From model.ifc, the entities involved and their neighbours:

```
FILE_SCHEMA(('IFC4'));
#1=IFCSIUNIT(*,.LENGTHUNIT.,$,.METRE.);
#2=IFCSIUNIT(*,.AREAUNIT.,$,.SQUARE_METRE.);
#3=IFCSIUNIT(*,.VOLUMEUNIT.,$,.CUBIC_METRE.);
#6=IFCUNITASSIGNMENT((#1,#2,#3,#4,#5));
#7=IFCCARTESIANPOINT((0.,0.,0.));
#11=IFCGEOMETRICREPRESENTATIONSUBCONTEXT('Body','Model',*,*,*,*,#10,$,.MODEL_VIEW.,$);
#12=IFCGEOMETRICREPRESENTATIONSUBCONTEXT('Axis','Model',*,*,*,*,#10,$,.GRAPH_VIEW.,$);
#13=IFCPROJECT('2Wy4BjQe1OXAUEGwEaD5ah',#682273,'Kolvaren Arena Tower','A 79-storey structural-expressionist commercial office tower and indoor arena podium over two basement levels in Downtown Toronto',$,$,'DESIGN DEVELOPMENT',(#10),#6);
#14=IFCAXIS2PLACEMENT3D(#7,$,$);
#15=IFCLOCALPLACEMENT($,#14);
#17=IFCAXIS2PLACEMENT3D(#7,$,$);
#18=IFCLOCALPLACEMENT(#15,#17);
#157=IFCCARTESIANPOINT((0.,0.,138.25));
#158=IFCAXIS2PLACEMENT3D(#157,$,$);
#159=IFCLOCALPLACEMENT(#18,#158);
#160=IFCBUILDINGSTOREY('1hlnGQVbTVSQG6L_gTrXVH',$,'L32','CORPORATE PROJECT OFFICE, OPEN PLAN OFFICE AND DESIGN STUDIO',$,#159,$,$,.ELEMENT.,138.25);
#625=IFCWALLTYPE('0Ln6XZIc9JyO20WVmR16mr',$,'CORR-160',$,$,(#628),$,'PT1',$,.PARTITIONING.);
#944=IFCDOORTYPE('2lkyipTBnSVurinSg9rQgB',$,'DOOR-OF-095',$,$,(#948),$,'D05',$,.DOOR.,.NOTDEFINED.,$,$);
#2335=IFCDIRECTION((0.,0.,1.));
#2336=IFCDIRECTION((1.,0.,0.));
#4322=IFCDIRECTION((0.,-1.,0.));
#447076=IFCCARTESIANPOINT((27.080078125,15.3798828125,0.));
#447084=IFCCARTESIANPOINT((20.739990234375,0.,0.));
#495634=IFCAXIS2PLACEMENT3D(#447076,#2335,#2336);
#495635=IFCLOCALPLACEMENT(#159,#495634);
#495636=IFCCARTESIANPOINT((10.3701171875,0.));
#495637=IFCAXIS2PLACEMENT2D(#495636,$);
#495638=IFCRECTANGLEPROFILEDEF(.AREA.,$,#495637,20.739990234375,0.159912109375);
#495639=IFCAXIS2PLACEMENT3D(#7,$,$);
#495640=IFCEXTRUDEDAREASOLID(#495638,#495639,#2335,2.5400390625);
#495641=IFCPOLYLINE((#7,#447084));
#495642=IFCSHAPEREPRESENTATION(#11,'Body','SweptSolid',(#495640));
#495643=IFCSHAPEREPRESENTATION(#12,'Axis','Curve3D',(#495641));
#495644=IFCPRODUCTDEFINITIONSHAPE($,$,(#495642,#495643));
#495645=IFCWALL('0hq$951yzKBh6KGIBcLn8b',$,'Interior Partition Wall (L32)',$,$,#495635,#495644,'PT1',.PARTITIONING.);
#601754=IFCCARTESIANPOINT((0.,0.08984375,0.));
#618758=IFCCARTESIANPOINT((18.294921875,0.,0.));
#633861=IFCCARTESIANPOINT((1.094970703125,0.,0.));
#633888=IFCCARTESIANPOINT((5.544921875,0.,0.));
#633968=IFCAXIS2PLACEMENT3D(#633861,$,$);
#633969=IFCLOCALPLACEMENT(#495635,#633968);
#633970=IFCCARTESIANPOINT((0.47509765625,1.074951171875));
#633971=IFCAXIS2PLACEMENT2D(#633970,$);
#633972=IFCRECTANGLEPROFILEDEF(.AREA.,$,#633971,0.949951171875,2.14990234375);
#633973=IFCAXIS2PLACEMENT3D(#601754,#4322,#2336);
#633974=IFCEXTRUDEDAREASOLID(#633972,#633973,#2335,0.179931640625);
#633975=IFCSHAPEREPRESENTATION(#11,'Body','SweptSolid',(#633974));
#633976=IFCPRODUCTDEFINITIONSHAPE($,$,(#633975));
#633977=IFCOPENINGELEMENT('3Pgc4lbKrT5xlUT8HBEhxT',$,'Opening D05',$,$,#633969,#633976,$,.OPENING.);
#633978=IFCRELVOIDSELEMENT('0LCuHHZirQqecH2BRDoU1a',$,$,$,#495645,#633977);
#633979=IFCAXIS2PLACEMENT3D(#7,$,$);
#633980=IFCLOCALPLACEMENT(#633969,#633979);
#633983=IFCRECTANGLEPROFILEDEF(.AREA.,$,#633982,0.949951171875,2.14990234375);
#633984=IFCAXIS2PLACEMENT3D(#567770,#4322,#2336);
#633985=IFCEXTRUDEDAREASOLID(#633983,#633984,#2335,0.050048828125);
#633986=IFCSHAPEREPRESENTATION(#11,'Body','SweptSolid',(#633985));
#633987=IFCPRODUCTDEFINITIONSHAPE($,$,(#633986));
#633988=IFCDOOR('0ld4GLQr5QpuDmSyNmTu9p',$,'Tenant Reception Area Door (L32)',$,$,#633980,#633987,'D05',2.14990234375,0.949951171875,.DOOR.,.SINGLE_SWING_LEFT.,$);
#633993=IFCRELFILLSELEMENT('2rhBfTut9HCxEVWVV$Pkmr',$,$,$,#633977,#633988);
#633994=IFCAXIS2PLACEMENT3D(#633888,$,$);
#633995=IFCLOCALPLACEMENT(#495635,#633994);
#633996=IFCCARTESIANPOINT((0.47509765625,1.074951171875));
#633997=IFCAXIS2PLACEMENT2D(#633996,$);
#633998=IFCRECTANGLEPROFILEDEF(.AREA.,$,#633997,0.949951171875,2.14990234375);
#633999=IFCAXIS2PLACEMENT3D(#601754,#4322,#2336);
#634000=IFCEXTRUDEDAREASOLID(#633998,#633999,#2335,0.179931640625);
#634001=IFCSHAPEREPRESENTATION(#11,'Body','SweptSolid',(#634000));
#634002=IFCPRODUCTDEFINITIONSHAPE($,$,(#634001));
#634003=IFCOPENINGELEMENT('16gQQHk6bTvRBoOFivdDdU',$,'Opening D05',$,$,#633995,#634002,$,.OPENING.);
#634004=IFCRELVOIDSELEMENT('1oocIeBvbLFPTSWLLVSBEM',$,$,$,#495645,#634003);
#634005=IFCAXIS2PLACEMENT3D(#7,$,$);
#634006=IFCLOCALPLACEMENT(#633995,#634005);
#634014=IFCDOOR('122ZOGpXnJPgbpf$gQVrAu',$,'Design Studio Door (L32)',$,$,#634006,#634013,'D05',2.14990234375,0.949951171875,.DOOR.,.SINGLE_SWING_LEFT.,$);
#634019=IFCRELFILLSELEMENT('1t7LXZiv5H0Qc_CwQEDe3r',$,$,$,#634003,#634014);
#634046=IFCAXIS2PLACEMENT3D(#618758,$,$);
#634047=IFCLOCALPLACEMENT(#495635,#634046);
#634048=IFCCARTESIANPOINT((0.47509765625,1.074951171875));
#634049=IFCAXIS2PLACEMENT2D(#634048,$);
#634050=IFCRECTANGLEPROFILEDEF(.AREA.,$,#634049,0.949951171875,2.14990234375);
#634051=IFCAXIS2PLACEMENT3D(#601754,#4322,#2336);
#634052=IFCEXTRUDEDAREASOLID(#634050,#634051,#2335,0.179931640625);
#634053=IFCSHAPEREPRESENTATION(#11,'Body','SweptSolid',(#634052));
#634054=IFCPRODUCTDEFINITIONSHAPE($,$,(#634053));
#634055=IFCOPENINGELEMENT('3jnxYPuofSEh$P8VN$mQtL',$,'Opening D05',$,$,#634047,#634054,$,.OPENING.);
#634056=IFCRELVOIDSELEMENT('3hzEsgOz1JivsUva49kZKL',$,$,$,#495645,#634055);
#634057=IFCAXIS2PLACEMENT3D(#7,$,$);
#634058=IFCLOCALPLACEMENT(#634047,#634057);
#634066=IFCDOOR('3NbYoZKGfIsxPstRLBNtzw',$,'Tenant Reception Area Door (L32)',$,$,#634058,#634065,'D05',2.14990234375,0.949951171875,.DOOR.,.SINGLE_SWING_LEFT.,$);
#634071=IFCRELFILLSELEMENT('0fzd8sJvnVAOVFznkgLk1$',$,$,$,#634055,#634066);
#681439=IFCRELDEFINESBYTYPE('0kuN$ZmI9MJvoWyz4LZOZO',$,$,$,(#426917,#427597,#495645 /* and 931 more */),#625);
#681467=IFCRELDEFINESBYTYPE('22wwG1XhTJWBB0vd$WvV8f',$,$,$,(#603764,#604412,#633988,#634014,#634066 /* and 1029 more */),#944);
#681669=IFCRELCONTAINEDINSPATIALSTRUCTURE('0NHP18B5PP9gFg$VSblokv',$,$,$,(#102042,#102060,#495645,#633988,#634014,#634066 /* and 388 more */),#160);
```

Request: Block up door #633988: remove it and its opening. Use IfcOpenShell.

```python
import ifcopenshell
import ifcopenshell.api.feature
import ifcopenshell.api.root
import ifcopenshell.geom
import ifcopenshell.util.shape

model = ifcopenshell.open("model.ifc")
settings = ifcopenshell.geom.settings()


def volume(element):
    """Net volume in cubic metres, openings subtracted."""
    shape = ifcopenshell.geom.create_shape(settings, element)
    return ifcopenshell.util.shape.get_volume(shape.geometry)


door = model.by_guid("0ld4GLQr5QpuDmSyNmTu9p")
opening = door.FillsVoids[0].RelatingOpeningElement
wall = opening.VoidsElements[0].RelatingBuildingElement
before = volume(wall)

ifcopenshell.api.root.remove_product(model, product=door)
ifcopenshell.api.feature.remove_feature(model, feature=opening)

after = volume(wall)

print(f"wall volume {before:.3f} -> {after:.3f} m3")

model.write("model-out.ifc")
```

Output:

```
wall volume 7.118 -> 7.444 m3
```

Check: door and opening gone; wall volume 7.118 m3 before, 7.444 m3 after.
